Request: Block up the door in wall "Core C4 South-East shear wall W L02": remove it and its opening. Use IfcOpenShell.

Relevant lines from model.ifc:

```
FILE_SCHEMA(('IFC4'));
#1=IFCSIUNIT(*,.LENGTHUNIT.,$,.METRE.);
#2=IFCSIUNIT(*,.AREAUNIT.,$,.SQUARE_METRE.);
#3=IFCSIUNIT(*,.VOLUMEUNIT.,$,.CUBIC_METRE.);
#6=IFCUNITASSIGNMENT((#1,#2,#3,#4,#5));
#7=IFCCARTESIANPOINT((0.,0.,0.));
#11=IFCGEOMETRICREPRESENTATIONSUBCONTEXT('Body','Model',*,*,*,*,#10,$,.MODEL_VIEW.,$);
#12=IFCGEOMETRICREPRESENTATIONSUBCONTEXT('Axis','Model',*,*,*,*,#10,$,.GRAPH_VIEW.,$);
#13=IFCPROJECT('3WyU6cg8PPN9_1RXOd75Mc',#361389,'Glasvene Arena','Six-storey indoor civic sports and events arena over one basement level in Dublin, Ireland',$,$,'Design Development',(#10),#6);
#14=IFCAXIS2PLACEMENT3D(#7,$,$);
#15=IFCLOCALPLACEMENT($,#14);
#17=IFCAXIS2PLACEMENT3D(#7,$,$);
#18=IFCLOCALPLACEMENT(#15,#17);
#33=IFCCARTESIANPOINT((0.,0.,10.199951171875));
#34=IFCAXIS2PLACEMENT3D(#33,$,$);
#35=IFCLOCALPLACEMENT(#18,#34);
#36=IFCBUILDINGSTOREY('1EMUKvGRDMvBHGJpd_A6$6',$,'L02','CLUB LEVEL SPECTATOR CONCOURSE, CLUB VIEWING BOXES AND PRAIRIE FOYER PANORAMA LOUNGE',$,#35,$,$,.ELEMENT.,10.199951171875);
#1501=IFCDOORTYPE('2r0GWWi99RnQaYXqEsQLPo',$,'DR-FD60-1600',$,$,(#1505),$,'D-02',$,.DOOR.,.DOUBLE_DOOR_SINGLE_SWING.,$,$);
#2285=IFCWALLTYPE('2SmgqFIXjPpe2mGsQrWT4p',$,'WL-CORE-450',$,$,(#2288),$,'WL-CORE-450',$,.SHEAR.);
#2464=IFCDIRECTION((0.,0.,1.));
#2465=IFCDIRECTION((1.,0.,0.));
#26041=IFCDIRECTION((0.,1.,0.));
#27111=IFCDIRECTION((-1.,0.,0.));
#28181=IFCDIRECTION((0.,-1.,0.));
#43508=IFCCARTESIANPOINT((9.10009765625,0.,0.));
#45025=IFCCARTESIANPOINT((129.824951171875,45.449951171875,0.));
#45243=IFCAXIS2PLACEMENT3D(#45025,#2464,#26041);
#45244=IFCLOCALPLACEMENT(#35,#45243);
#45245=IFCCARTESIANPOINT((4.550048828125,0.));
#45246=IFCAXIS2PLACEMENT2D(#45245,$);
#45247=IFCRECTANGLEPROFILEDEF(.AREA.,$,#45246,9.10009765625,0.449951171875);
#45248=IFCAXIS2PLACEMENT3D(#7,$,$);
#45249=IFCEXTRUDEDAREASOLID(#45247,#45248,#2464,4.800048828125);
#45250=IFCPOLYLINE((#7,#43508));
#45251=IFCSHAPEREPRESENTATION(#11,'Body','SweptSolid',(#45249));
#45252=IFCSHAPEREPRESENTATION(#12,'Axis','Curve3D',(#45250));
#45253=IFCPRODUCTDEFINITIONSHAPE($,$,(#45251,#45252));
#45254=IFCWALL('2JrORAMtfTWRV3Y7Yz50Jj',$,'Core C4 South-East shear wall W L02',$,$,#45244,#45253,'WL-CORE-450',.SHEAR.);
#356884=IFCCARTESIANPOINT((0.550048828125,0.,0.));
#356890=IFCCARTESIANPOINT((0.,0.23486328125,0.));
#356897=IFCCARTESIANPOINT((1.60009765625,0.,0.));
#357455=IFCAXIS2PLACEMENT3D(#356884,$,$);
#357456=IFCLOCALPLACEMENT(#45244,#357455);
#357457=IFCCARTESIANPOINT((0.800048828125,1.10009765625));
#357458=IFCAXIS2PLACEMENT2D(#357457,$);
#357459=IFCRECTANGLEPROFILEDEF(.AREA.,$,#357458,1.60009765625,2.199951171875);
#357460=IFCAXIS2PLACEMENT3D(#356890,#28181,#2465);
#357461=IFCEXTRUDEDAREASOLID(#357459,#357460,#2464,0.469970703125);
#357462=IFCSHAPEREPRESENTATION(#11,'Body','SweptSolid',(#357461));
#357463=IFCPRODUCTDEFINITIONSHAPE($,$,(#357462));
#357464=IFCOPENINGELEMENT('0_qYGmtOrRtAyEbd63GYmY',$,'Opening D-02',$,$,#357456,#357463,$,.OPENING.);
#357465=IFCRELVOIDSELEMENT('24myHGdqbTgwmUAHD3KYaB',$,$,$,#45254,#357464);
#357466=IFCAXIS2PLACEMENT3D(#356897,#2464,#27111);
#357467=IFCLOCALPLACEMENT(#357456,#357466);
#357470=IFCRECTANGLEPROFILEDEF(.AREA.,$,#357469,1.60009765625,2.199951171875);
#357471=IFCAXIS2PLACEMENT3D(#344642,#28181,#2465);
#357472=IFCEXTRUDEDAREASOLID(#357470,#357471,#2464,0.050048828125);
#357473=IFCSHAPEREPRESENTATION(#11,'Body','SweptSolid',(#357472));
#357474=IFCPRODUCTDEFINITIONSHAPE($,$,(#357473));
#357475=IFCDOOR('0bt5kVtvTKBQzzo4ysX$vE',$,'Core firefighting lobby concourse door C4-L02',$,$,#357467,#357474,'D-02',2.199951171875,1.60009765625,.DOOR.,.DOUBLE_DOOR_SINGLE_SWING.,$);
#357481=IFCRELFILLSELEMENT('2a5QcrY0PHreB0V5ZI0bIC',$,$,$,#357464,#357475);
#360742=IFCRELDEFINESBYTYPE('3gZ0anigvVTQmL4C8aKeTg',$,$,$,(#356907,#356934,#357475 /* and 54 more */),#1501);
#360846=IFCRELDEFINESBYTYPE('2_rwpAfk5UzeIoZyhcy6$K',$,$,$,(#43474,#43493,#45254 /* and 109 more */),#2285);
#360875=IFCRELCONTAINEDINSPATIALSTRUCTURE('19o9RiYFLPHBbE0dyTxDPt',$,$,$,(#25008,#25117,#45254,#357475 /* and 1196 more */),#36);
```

```python
import ifcopenshell
import ifcopenshell.api.feature
import ifcopenshell.api.root
import ifcopenshell.geom
import ifcopenshell.util.shape

model = ifcopenshell.open("model.ifc")
settings = ifcopenshell.geom.settings()


def volume(element):
    """Net volume in cubic metres, openings subtracted."""
    shape = ifcopenshell.geom.create_shape(settings, element)
    return ifcopenshell.util.shape.get_volume(shape.geometry)


door = model.by_guid("0bt5kVtvTKBQzzo4ysX$vE")
opening = door.FillsVoids[0].RelatingOpeningElement
wall = opening.VoidsElements[0].RelatingBuildingElement
before = volume(wall)

ifcopenshell.api.root.remove_product(model, product=door)
ifcopenshell.api.feature.remove_feature(model, feature=opening)

after = volume(wall)

print(f"wall volume {before:.3f} -> {after:.3f} m3")

model.write("model_updated.ifc")
```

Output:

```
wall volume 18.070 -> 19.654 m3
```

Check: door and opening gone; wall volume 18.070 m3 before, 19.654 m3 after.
